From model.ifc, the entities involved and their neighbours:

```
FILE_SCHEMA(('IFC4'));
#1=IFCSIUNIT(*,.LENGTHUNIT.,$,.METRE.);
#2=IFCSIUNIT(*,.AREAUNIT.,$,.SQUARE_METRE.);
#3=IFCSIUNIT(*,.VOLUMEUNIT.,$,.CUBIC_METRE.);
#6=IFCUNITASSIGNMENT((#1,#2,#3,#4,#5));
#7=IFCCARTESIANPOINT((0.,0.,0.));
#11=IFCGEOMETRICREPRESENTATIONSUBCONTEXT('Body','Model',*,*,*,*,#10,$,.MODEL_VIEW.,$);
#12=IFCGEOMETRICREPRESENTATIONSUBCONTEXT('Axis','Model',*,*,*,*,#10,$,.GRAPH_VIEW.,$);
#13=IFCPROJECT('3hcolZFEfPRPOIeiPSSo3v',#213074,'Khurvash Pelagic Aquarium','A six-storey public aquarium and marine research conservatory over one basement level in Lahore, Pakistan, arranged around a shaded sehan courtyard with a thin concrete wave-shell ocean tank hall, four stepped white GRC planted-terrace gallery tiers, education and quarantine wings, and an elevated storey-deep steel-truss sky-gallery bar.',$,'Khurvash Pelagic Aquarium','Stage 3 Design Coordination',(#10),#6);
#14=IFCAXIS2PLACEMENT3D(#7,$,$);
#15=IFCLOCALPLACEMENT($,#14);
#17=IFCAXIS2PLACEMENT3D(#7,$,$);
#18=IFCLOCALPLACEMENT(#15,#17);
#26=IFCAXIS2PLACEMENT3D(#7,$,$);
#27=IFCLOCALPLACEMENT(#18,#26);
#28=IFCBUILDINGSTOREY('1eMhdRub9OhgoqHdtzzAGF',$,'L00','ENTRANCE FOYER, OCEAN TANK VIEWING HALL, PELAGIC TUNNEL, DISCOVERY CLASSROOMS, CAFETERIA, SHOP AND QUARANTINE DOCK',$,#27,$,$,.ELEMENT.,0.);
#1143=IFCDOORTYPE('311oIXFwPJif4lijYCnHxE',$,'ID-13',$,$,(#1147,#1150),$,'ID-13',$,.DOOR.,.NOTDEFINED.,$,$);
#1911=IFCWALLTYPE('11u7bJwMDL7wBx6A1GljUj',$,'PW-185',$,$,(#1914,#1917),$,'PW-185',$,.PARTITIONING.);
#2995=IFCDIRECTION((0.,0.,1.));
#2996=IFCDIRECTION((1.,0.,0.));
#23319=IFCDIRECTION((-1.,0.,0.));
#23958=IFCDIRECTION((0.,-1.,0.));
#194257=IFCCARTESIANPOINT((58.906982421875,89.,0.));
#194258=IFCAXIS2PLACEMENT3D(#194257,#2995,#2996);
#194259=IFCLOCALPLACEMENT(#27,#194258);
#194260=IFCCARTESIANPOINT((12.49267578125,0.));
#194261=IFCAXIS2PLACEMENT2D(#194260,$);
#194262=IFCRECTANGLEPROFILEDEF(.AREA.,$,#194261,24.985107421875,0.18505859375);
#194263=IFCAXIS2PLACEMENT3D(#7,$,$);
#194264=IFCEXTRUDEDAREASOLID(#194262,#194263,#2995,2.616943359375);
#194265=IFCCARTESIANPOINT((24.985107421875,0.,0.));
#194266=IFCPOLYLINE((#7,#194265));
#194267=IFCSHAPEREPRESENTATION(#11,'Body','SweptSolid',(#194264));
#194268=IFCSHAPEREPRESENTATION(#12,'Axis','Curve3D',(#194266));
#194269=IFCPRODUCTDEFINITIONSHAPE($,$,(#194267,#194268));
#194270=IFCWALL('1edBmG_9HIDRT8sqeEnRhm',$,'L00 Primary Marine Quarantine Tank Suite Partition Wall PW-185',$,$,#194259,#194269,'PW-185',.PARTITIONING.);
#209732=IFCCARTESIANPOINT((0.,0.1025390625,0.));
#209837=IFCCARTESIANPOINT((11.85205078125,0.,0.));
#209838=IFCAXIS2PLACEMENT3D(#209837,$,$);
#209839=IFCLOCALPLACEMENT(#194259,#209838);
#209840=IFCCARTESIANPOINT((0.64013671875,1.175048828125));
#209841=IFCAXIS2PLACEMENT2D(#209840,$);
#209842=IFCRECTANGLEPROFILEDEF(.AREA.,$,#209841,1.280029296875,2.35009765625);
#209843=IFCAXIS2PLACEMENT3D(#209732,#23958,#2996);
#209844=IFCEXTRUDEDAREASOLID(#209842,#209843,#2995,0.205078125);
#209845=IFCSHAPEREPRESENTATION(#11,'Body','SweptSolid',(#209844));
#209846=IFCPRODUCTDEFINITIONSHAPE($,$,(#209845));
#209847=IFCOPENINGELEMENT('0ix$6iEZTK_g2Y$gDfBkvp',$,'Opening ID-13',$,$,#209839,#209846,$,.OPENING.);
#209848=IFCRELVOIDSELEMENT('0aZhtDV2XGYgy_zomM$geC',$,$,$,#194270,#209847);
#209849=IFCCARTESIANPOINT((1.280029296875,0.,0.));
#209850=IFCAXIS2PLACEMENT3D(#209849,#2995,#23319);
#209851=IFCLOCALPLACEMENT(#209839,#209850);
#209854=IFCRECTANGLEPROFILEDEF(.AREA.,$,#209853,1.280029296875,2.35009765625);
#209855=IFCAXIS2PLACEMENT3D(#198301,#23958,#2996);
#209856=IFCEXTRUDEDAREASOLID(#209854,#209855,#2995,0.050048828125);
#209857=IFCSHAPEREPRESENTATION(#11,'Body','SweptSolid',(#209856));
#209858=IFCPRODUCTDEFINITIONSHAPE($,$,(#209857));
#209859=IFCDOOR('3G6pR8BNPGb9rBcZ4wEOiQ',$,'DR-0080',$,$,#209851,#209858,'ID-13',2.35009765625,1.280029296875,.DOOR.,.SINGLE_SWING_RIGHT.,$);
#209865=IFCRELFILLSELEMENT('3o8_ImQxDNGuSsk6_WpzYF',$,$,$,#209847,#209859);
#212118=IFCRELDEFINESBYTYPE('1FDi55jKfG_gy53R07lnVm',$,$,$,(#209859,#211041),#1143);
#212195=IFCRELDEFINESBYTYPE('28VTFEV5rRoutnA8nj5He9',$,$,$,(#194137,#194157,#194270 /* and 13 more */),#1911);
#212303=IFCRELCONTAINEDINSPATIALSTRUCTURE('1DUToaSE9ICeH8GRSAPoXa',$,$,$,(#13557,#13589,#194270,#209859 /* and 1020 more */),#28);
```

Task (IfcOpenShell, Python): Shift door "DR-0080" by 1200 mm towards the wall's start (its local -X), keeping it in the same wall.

```python
import ifcopenshell
import ifcopenshell.api.geometry
import ifcopenshell.util.placement
import ifcopenshell.util.unit

model = ifcopenshell.open("model.ifc")
unit_scale = ifcopenshell.util.unit.calculate_unit_scale(model)

door = model.by_guid("3G6pR8BNPGb9rBcZ4wEOiQ")
opening = door.FillsVoids[0].RelatingOpeningElement
wall = opening.VoidsElements[0].RelatingBuildingElement

wall_matrix = ifcopenshell.util.placement.get_local_placement(wall.ObjectPlacement)
shift = wall_matrix[:3, 0] * -1.2 / unit_scale
before = ifcopenshell.util.placement.get_local_placement(door.ObjectPlacement)[:3, 3].copy()

# The door is placed relative to its opening, so it follows when the opening moves.
matrix = ifcopenshell.util.placement.get_local_placement(opening.ObjectPlacement)
matrix[:3, 3] += shift
ifcopenshell.api.geometry.edit_object_placement(
    model, product=opening, matrix=matrix, is_si=False, should_transform_children=True
)

after = ifcopenshell.util.placement.get_local_placement(door.ObjectPlacement)[:3, 3]
print("door moved by", (after - before).round(3) + 0.0)

model.write("model_edited.ifc")
```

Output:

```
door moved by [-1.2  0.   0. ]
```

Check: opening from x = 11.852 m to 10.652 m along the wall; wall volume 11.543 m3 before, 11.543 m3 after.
